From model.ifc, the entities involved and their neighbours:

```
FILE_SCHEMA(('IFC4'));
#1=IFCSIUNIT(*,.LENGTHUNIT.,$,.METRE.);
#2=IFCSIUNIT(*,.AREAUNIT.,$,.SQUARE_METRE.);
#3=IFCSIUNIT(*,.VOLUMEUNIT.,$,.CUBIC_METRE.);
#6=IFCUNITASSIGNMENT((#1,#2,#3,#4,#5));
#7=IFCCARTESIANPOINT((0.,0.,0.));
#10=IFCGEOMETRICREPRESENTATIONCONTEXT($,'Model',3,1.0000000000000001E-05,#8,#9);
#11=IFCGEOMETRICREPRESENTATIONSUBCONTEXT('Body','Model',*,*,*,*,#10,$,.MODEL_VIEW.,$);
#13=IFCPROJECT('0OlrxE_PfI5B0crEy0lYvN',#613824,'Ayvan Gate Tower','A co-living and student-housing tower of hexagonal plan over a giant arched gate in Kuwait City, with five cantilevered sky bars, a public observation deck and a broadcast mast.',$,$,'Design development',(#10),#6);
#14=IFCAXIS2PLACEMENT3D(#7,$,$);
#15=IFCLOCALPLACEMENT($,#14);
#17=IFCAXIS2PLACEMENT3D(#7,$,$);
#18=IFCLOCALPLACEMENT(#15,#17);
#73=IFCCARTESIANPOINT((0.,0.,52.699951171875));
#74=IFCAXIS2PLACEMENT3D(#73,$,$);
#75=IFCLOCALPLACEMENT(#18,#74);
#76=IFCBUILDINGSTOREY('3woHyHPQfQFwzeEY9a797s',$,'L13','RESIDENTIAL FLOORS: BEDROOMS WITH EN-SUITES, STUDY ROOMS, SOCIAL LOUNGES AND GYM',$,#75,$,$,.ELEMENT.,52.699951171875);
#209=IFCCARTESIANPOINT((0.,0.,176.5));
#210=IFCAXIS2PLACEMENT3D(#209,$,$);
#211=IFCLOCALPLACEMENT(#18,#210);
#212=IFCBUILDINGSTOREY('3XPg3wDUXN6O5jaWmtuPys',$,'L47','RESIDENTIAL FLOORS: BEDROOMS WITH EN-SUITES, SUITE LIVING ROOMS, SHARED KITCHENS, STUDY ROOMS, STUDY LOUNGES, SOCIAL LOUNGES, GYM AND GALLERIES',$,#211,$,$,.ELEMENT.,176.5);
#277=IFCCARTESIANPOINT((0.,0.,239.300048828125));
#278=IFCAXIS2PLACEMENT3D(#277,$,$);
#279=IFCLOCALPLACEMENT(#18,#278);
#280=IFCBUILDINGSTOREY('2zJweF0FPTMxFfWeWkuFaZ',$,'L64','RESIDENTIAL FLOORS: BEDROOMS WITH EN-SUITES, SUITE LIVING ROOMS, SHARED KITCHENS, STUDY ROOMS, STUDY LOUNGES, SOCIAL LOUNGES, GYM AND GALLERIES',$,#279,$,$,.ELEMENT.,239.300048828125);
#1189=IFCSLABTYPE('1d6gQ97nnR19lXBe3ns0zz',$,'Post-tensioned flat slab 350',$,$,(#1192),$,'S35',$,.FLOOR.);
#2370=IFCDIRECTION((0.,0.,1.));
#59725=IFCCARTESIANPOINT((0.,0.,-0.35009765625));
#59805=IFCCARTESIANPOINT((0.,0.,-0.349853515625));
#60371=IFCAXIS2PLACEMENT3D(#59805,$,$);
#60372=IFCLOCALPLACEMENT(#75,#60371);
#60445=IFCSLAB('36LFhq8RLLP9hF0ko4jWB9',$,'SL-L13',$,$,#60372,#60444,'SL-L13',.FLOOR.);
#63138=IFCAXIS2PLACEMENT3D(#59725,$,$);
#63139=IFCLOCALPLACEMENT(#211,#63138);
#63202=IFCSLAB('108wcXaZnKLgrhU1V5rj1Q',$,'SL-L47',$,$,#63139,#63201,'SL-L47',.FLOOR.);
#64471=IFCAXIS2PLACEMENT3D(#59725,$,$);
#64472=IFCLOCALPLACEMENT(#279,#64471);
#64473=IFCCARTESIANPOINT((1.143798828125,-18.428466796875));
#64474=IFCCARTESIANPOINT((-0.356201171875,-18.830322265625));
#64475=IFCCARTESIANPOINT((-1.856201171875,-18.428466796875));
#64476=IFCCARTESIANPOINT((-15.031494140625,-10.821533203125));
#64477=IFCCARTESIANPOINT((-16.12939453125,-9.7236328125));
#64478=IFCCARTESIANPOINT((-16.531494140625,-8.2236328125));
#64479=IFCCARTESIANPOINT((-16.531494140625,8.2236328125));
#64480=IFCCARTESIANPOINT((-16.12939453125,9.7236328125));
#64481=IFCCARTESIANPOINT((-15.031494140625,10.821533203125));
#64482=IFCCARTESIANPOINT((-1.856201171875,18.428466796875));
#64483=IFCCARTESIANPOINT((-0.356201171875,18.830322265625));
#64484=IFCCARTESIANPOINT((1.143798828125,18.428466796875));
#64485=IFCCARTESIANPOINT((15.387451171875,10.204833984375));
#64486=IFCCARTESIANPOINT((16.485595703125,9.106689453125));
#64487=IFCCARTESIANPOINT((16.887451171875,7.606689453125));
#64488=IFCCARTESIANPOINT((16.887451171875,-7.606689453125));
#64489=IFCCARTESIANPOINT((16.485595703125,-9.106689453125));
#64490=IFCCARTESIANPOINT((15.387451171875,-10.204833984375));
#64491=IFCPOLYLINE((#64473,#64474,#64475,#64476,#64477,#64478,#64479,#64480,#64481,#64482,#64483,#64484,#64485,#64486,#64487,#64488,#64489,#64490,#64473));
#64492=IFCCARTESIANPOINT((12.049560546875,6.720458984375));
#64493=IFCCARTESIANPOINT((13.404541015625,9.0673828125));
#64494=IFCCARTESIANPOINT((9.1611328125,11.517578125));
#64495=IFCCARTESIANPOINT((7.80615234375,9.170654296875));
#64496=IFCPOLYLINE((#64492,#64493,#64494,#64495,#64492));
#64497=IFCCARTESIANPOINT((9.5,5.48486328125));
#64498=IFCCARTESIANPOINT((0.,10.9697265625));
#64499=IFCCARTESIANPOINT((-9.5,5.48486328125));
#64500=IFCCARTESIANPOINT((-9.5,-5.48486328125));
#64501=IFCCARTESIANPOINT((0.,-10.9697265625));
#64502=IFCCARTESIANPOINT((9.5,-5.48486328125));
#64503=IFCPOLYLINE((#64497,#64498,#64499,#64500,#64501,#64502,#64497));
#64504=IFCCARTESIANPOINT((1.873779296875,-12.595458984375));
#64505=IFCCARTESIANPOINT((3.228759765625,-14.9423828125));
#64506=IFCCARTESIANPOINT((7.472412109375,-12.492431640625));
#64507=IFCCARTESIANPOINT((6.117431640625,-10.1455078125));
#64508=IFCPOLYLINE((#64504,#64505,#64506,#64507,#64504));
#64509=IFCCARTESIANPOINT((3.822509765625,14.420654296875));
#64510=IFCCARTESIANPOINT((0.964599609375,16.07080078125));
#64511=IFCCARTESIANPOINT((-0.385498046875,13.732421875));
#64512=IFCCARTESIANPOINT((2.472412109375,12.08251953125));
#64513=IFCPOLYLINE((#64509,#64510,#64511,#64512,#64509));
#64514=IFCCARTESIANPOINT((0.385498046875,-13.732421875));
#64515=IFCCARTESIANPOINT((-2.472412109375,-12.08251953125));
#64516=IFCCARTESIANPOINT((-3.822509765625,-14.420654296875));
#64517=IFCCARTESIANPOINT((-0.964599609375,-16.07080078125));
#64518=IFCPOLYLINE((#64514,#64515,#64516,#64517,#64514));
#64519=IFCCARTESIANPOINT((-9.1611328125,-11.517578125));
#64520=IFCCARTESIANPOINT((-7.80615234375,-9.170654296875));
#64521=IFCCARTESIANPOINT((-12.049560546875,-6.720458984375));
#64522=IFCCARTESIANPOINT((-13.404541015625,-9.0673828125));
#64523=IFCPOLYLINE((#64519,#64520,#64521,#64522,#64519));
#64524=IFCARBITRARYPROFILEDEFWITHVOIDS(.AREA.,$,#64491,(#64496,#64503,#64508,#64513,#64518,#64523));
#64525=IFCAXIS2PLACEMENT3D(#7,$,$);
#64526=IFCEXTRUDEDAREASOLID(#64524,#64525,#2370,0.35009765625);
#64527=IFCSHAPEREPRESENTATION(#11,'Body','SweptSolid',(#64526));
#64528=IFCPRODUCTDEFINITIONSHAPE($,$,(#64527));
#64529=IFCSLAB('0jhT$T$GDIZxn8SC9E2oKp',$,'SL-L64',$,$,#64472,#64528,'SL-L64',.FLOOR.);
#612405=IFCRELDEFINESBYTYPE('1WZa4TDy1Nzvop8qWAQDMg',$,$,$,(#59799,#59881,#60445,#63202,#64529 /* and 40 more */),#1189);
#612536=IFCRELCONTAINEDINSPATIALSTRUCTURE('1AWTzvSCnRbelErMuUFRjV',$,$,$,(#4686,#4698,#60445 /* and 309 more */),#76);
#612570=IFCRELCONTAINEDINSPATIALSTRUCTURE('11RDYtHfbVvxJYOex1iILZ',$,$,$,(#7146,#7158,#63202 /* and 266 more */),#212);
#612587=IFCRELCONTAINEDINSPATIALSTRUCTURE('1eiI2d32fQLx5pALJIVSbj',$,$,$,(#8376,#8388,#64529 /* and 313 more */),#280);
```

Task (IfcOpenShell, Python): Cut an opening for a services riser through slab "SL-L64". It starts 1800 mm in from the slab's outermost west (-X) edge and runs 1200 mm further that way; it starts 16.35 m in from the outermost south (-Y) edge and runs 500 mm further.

```python
import numpy as np
import ifcopenshell
import ifcopenshell.api.feature
import ifcopenshell.api.geometry
import ifcopenshell.api.root
import ifcopenshell.geom
import ifcopenshell.util.placement
import ifcopenshell.util.representation
import ifcopenshell.util.shape
import ifcopenshell.util.unit

model = ifcopenshell.open("model.ifc")
unit_scale = ifcopenshell.util.unit.calculate_unit_scale(model)
settings = ifcopenshell.geom.settings()


def volume(element):
    """Net volume in cubic metres, openings subtracted."""
    shape = ifcopenshell.geom.create_shape(settings, element)
    return ifcopenshell.util.shape.get_volume(shape.geometry)


slab = model.by_guid("0jhT$T$GDIZxn8SC9E2oKp")
before = volume(slab)

# Extent in the slab's own axes, in metres. The edges named are its -X and -Y sides.
slab_shape = ifcopenshell.geom.create_shape(settings, slab)
vertices = ifcopenshell.util.shape.get_vertices(slab_shape.geometry)
x_min, y_min, bottom = vertices.min(axis=0)
top = vertices[:, 2].max()

opening = ifcopenshell.api.root.create_entity(model, ifc_class="IfcOpeningElement", name="Services riser opening", predefined_type="OPENING")
context = ifcopenshell.util.representation.get_context(model, "Model", "Body", "MODEL_VIEW")
width, depth = 1.2, 0.5
outline = [(0.0, 0.0), (width, 0.0), (width, depth), (0.0, depth), (0.0, 0.0)]
# Overshoot both faces by 50 mm so the cut is clean.
shape = ifcopenshell.api.geometry.add_slab_representation(
    model, context=context, depth=top - bottom + 0.1, polyline=outline
)
ifcopenshell.api.geometry.assign_representation(model, product=opening, representation=shape)

matrix = ifcopenshell.util.placement.get_local_placement(slab.ObjectPlacement)
matrix[:, 3] = matrix @ np.append(np.array([x_min + 1.8, y_min + 16.35, bottom - 0.05]) / unit_scale, 1.0)
ifcopenshell.api.geometry.edit_object_placement(model, product=opening, matrix=matrix, is_si=False)
ifcopenshell.api.feature.add_feature(model, feature=opening, element=slab)

after = volume(slab)

print(f"slab volume {before:.3f} -> {after:.3f} m3")

model.write("model-out.ifc")
```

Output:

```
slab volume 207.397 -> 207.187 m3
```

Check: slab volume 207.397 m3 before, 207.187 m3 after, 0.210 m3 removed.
